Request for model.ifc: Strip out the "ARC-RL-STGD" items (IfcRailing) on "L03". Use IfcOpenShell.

First a look at what the model holds.

```python
import ifcopenshell
import ifcopenshell.util.element

model = ifcopenshell.open("model.ifc")
print(model.schema)
storey = next(s for s in model.by_type("IfcBuildingStorey") if s.Name == "L03")
railings = [e for e in ifcopenshell.util.element.get_decomposition(storey) if e.is_a("IfcRailing")]
seen = {}
for e in railings:
    element_type = ifcopenshell.util.element.get_type(e)
    name = element_type.Name if element_type not in (None, e) else None
    seen[name] = seen.get(name, 0) + 1
for name, count in sorted(seen.items(), key=str):
    print(count, "x", name)
```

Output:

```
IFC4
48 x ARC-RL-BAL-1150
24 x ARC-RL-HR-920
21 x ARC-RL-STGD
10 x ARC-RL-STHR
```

```python
import ifcopenshell
import ifcopenshell.api.root
import ifcopenshell.util.element

model = ifcopenshell.open("model.ifc")

storey = next(s for s in model.by_type("IfcBuildingStorey") if s.Name == "L03")
railings = [e for e in ifcopenshell.util.element.get_decomposition(storey) if e.is_a("IfcRailing")]
targets = [e for e in railings if (t := ifcopenshell.util.element.get_type(e)) not in (None, e) and t.Name == "ARC-RL-STGD"]

for e in targets:
    ifcopenshell.api.root.remove_product(model, product=e)
print(len(targets), "removed")

model.write("model_edited.ifc")
```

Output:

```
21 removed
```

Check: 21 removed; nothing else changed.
